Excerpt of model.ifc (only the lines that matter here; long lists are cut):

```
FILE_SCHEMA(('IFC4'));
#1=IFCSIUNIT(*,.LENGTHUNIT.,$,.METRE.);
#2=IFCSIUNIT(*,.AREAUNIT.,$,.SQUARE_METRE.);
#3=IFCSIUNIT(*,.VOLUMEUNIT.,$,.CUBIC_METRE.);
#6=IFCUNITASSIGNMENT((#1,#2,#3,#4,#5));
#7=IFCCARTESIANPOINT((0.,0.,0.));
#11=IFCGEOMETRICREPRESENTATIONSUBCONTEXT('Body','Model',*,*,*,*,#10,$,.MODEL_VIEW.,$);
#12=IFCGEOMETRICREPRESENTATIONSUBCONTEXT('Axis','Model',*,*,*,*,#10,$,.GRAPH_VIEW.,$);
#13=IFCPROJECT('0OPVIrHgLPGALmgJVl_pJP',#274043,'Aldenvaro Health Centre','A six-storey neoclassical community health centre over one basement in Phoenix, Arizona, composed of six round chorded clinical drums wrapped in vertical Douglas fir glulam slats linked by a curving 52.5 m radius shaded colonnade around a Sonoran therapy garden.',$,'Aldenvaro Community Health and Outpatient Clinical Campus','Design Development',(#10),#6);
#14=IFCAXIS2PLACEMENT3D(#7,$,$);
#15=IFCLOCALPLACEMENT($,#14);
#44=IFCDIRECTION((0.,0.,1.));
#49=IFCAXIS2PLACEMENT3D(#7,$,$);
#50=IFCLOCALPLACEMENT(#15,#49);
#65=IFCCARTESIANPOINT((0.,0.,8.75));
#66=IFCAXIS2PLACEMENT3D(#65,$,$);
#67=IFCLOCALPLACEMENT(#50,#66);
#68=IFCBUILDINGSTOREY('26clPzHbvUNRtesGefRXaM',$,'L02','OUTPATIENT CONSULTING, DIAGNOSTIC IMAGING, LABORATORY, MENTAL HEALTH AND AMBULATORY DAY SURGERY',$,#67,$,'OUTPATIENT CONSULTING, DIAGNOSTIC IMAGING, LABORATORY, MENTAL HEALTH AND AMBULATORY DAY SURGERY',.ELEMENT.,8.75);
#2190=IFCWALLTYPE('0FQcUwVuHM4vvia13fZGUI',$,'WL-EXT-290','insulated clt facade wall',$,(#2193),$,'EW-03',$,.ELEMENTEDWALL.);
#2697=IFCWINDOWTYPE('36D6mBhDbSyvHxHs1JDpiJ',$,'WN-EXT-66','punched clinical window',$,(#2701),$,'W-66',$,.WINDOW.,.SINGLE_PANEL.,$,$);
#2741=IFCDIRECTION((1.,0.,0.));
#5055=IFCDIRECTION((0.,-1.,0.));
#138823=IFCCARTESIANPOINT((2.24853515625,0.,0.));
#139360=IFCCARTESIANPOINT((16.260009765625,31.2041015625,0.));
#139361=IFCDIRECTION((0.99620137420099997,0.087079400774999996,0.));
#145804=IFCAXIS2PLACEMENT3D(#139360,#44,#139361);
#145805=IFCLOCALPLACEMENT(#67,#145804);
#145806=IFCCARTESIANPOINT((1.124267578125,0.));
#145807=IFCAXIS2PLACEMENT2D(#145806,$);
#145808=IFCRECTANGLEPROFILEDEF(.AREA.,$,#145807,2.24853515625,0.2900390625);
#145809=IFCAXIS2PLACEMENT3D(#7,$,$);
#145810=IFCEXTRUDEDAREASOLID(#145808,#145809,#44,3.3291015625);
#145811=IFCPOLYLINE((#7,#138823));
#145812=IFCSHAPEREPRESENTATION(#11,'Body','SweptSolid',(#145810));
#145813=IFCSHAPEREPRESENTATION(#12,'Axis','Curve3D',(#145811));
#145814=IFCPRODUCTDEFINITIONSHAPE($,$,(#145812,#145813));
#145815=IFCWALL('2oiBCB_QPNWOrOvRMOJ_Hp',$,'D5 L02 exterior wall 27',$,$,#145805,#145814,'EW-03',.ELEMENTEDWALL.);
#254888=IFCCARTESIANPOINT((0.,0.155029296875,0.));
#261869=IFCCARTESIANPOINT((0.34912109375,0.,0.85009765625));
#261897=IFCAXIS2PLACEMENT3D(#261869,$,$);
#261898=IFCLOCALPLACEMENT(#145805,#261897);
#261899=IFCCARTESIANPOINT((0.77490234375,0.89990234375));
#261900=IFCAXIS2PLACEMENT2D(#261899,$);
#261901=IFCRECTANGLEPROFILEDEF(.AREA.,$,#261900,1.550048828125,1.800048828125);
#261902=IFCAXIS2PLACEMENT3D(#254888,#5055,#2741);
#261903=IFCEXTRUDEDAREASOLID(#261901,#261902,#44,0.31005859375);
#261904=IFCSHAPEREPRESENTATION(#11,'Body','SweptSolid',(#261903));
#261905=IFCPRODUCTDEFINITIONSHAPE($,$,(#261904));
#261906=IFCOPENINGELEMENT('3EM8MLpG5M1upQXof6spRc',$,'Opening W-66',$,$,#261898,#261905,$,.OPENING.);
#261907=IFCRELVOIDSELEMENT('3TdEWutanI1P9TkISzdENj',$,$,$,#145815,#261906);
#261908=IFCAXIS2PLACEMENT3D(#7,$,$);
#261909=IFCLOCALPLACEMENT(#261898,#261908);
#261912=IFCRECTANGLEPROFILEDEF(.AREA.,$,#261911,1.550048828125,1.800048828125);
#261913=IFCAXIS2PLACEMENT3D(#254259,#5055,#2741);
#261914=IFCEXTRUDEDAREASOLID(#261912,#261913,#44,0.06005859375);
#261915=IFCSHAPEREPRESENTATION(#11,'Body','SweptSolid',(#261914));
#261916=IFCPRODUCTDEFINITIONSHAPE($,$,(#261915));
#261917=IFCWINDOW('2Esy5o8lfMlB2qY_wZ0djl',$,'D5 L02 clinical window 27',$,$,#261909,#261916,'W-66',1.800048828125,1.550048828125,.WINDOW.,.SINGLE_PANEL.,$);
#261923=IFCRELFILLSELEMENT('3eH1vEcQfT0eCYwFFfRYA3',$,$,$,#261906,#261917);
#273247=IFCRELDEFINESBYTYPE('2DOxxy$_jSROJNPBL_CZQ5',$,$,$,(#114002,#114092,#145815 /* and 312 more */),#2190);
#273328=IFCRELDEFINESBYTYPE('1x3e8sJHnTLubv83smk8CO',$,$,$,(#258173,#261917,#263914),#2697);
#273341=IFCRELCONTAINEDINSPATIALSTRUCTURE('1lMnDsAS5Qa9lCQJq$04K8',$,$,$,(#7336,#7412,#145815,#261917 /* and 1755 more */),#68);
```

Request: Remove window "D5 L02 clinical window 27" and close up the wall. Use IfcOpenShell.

```python
import ifcopenshell
import ifcopenshell.api.feature
import ifcopenshell.api.root
import ifcopenshell.geom
import ifcopenshell.util.shape

model = ifcopenshell.open("model.ifc")
settings = ifcopenshell.geom.settings()


def volume(element):
    """Net volume in cubic metres, openings subtracted."""
    shape = ifcopenshell.geom.create_shape(settings, element)
    return ifcopenshell.util.shape.get_volume(shape.geometry)


window = model.by_guid("2Esy5o8lfMlB2qY_wZ0djl")
opening = window.FillsVoids[0].RelatingOpeningElement
wall = opening.VoidsElements[0].RelatingBuildingElement
before = volume(wall)

ifcopenshell.api.root.remove_product(model, product=window)
ifcopenshell.api.feature.remove_feature(model, feature=opening)

after = volume(wall)

print(f"wall volume {before:.3f} -> {after:.3f} m3")

model.write("model_updated.ifc")
```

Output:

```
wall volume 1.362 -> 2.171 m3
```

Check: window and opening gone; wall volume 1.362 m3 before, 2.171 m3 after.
